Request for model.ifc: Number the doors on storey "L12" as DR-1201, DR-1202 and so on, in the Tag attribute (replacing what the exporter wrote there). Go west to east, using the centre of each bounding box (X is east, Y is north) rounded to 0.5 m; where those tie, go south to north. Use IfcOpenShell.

First a look at what the model holds.

```python
import ifcopenshell
import ifcopenshell.util.element
import ifcopenshell.util.placement

model = ifcopenshell.open("model.ifc")
print(model.schema)
storey = next(s for s in model.by_type("IfcBuildingStorey") if s.Name == "L12")
doors = [e for e in ifcopenshell.util.element.get_decomposition(storey) if e.is_a("IfcDoor")]
for e in sorted(doors, key=lambda e: e.id()):
    origin = ifcopenshell.util.placement.get_local_placement(e.ObjectPlacement)[:3, 3]
    print(e.id(), e.Tag, e.Name, origin.round(2) + 0.0, sep=" | ")
```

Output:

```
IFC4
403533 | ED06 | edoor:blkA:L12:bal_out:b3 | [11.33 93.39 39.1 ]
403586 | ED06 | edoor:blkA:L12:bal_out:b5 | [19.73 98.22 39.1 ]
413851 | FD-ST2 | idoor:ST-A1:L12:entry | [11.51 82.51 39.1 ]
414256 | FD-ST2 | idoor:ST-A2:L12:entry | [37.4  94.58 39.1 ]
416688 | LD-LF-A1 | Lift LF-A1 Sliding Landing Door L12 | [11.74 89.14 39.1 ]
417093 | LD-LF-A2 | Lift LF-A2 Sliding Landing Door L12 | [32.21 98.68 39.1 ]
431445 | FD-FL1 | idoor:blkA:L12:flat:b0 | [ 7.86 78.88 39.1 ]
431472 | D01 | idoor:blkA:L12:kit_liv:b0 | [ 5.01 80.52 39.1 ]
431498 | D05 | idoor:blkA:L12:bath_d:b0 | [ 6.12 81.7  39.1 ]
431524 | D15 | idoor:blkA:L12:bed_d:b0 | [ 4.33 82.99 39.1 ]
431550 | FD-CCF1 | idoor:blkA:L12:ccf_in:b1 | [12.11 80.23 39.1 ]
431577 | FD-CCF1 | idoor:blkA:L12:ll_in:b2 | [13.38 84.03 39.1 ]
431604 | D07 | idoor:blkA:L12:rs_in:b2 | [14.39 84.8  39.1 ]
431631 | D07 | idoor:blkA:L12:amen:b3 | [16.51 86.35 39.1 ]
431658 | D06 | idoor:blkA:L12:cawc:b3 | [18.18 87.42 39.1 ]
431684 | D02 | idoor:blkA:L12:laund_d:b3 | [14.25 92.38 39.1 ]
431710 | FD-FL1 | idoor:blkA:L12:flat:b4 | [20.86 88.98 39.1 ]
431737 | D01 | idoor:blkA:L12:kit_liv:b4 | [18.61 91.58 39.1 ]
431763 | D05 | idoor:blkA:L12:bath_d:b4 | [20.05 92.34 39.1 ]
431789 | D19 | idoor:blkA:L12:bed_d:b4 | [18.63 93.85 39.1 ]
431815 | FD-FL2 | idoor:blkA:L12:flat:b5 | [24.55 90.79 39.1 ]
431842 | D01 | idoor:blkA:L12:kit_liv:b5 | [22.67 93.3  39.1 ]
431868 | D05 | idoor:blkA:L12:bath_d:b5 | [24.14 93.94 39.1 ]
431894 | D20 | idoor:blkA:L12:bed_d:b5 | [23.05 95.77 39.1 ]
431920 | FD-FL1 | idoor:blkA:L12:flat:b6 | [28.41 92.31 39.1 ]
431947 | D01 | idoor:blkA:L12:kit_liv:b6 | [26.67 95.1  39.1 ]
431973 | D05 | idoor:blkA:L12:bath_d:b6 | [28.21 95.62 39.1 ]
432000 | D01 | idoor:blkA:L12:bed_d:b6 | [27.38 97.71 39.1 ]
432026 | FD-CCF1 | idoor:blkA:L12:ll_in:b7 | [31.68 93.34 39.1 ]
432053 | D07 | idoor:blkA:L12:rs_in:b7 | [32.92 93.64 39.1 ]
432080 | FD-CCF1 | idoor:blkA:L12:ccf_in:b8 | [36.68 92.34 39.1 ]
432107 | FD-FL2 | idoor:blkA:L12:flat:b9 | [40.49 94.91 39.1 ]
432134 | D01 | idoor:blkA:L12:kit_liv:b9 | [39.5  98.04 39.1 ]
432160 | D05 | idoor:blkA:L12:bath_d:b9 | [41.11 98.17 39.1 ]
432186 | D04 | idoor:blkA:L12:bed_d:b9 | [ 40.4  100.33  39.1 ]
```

```python
import ifcopenshell
import ifcopenshell.geom
import ifcopenshell.util.element
import ifcopenshell.util.shape

model = ifcopenshell.open("model.ifc")
settings = ifcopenshell.geom.settings()
settings.set("use-world-coords", True)


def centre(element):
    shape = ifcopenshell.geom.create_shape(settings, element)
    return ifcopenshell.util.shape.get_bbox_centroid(shape.geometry)


storey = next(s for s in model.by_type("IfcBuildingStorey") if s.Name == "L12")
doors = [e for e in ifcopenshell.util.element.get_decomposition(storey) if e.is_a("IfcDoor")]

# Insertion points can sit at a corner or the storey origin, so sort by the geometry (in metres).
centres = {e: centre(e) for e in doors}
doors.sort(key=lambda e: (round(centres[e][0] / 0.5), centres[e][1]))

for i, e in enumerate(doors, start=1):
    number = f"DR-12{i:02d}"
    e.Tag = number
    print(e.id(), number)

model.write("model_edited.ifc")
```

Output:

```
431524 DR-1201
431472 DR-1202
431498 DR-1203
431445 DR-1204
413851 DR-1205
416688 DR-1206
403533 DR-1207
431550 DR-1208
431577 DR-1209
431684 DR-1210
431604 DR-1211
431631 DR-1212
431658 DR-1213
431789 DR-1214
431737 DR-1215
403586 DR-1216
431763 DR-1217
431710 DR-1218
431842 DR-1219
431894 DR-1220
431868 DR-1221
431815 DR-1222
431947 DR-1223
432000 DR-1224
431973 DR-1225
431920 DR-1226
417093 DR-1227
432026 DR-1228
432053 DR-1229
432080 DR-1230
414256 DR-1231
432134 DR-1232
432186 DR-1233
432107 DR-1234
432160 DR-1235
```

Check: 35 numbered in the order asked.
